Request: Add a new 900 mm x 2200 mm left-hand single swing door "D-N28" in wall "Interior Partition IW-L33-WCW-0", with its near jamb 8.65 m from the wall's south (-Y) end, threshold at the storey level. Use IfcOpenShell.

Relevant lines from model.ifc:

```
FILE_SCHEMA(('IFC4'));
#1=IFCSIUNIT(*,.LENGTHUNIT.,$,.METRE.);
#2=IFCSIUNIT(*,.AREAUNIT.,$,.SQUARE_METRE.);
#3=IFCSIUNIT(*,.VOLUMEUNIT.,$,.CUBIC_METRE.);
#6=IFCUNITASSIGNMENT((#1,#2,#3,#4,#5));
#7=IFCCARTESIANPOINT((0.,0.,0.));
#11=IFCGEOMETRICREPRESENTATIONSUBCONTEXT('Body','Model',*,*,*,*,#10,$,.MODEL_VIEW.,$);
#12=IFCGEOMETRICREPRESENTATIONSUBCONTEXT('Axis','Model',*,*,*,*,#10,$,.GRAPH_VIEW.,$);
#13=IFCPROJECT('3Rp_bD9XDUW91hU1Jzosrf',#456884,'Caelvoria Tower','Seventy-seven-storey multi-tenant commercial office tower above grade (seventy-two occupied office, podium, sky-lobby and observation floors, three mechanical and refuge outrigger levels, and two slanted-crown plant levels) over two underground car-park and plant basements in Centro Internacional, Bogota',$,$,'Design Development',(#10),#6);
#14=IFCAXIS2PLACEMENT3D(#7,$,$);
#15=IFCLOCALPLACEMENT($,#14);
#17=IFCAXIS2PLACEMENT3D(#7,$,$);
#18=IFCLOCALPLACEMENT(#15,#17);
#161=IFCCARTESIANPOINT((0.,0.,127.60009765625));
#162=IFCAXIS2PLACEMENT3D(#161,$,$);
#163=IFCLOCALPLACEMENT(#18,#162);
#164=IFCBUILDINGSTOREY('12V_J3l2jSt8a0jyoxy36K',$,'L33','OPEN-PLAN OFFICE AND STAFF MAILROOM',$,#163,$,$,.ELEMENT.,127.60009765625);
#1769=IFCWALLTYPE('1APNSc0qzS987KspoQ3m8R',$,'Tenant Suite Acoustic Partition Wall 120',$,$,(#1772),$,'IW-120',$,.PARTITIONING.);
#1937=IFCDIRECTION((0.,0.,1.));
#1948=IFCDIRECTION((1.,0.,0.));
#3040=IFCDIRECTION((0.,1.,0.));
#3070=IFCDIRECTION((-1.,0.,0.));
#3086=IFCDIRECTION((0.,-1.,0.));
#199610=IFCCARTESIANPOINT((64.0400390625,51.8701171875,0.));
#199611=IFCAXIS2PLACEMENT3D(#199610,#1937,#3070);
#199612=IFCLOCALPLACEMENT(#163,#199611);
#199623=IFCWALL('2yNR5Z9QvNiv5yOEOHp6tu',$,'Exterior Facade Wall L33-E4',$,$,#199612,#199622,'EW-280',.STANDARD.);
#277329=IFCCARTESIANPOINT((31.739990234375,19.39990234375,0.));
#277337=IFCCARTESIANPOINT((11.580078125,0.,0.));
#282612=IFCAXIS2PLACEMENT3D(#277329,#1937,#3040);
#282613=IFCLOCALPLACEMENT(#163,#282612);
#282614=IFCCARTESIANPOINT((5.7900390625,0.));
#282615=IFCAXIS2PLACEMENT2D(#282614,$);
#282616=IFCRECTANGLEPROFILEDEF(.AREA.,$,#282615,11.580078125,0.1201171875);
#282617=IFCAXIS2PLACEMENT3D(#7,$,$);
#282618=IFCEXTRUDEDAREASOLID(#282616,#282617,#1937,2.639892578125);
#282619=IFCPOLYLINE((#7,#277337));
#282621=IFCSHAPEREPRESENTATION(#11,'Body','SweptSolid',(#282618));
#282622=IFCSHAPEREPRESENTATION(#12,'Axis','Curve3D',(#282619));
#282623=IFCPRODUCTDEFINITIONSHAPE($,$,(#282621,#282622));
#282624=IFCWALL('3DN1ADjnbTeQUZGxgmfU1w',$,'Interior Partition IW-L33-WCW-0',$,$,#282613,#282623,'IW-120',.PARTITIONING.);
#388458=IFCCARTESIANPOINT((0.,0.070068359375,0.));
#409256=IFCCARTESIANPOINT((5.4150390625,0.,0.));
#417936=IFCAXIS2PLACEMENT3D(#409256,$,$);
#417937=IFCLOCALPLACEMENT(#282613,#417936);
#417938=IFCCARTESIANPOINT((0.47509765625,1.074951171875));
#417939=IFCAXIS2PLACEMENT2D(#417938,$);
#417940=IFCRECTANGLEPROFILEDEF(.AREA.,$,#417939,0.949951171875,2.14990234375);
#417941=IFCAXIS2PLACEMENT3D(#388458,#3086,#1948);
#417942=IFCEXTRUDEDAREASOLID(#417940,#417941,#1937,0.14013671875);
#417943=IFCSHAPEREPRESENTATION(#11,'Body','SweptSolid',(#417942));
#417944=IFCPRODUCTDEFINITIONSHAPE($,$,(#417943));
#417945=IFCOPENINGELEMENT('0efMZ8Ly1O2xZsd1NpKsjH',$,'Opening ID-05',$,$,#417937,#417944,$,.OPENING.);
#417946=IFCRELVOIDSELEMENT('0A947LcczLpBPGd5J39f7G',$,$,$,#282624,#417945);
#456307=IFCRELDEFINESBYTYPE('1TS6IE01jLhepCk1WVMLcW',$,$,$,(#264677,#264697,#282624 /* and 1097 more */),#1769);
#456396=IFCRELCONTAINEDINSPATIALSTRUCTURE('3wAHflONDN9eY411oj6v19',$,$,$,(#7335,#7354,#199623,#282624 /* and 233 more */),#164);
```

```python
import numpy as np
import ifcopenshell
import ifcopenshell.api.feature
import ifcopenshell.api.geometry
import ifcopenshell.api.root
import ifcopenshell.api.spatial
import ifcopenshell.geom
import ifcopenshell.util.element
import ifcopenshell.util.placement
import ifcopenshell.util.representation
import ifcopenshell.util.shape
import ifcopenshell.util.unit

model = ifcopenshell.open("model.ifc")
unit_scale = ifcopenshell.util.unit.calculate_unit_scale(model)
settings = ifcopenshell.geom.settings()


def volume(element):
    """Net volume in cubic metres, openings subtracted."""
    shape = ifcopenshell.geom.create_shape(settings, element)
    return ifcopenshell.util.shape.get_volume(shape.geometry)


wall = model.by_guid("3DN1ADjnbTeQUZGxgmfU1w")
storey = ifcopenshell.util.element.get_container(wall, ifc_class="IfcBuildingStorey")
context = ifcopenshell.util.representation.get_context(model, "Model", "Body", "MODEL_VIEW")
before = volume(wall)

width, height, from_end, sill = 0.9, 2.2, 8.65, 0.0  # metres

# The wall runs along its own X axis, and the end named is its -X end.
wall_shape = ifcopenshell.geom.create_shape(settings, wall)
x, y, z = ifcopenshell.util.shape.get_vertices(wall_shape.geometry).T
start = x.min() + from_end
face, thickness = float(y.min()), float(y.max() - y.min())
wall_matrix = ifcopenshell.util.placement.get_local_placement(wall.ObjectPlacement)
level = ifcopenshell.util.placement.get_local_placement(storey.ObjectPlacement)[2, 3]


def in_wall(x, y):
    """Placement at x, y metres in the wall's axes, at sill height."""
    matrix = wall_matrix.copy()
    matrix[:, 3] = wall_matrix @ np.array([x / unit_scale, y / unit_scale, 0.0, 1.0])
    matrix[2, 3] = level + sill / unit_scale
    return matrix


# Opening: a box that overshoots both wall faces by 50 mm.
opening = ifcopenshell.api.root.create_entity(model, ifc_class="IfcOpeningElement", predefined_type="OPENING")
box = ifcopenshell.api.geometry.add_wall_representation(
    model, context=context, length=width, height=height, thickness=thickness + 0.1
)
ifcopenshell.api.geometry.assign_representation(model, product=opening, representation=box)
ifcopenshell.api.geometry.edit_object_placement(model, product=opening, matrix=in_wall(start, face - 0.05), is_si=False)
ifcopenshell.api.feature.add_feature(model, feature=opening, element=wall)

door = ifcopenshell.api.root.create_entity(model, ifc_class="IfcDoor", name="D-N28", predefined_type="DOOR")
door.OverallWidth, door.OverallHeight = width / unit_scale, height / unit_scale
door.OperationType = "SINGLE_SWING_LEFT"
body = ifcopenshell.api.geometry.add_door_representation(
    model,
    context=context,
    overall_width=door.OverallWidth,
    overall_height=door.OverallHeight,
    operation_type="SINGLE_SWING_LEFT",
    lining_properties={"LiningDepth": thickness / unit_scale, "ThresholdDepth": thickness / unit_scale},
)
ifcopenshell.api.geometry.assign_representation(model, product=door, representation=body)
ifcopenshell.api.spatial.assign_container(model, products=[door], relating_structure=storey)
ifcopenshell.api.feature.add_filling(model, opening=opening, element=door)

# The lining spans the wall, so the door starts at the wall face.
ifcopenshell.api.geometry.edit_object_placement(model, product=door, matrix=in_wall(start, face), is_si=False)

after = volume(wall)

print(f"wall volume {before:.3f} -> {after:.3f} m3")

model.write("model_updated.ifc")
```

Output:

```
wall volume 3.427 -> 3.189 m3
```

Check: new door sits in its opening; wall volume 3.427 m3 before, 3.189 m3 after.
